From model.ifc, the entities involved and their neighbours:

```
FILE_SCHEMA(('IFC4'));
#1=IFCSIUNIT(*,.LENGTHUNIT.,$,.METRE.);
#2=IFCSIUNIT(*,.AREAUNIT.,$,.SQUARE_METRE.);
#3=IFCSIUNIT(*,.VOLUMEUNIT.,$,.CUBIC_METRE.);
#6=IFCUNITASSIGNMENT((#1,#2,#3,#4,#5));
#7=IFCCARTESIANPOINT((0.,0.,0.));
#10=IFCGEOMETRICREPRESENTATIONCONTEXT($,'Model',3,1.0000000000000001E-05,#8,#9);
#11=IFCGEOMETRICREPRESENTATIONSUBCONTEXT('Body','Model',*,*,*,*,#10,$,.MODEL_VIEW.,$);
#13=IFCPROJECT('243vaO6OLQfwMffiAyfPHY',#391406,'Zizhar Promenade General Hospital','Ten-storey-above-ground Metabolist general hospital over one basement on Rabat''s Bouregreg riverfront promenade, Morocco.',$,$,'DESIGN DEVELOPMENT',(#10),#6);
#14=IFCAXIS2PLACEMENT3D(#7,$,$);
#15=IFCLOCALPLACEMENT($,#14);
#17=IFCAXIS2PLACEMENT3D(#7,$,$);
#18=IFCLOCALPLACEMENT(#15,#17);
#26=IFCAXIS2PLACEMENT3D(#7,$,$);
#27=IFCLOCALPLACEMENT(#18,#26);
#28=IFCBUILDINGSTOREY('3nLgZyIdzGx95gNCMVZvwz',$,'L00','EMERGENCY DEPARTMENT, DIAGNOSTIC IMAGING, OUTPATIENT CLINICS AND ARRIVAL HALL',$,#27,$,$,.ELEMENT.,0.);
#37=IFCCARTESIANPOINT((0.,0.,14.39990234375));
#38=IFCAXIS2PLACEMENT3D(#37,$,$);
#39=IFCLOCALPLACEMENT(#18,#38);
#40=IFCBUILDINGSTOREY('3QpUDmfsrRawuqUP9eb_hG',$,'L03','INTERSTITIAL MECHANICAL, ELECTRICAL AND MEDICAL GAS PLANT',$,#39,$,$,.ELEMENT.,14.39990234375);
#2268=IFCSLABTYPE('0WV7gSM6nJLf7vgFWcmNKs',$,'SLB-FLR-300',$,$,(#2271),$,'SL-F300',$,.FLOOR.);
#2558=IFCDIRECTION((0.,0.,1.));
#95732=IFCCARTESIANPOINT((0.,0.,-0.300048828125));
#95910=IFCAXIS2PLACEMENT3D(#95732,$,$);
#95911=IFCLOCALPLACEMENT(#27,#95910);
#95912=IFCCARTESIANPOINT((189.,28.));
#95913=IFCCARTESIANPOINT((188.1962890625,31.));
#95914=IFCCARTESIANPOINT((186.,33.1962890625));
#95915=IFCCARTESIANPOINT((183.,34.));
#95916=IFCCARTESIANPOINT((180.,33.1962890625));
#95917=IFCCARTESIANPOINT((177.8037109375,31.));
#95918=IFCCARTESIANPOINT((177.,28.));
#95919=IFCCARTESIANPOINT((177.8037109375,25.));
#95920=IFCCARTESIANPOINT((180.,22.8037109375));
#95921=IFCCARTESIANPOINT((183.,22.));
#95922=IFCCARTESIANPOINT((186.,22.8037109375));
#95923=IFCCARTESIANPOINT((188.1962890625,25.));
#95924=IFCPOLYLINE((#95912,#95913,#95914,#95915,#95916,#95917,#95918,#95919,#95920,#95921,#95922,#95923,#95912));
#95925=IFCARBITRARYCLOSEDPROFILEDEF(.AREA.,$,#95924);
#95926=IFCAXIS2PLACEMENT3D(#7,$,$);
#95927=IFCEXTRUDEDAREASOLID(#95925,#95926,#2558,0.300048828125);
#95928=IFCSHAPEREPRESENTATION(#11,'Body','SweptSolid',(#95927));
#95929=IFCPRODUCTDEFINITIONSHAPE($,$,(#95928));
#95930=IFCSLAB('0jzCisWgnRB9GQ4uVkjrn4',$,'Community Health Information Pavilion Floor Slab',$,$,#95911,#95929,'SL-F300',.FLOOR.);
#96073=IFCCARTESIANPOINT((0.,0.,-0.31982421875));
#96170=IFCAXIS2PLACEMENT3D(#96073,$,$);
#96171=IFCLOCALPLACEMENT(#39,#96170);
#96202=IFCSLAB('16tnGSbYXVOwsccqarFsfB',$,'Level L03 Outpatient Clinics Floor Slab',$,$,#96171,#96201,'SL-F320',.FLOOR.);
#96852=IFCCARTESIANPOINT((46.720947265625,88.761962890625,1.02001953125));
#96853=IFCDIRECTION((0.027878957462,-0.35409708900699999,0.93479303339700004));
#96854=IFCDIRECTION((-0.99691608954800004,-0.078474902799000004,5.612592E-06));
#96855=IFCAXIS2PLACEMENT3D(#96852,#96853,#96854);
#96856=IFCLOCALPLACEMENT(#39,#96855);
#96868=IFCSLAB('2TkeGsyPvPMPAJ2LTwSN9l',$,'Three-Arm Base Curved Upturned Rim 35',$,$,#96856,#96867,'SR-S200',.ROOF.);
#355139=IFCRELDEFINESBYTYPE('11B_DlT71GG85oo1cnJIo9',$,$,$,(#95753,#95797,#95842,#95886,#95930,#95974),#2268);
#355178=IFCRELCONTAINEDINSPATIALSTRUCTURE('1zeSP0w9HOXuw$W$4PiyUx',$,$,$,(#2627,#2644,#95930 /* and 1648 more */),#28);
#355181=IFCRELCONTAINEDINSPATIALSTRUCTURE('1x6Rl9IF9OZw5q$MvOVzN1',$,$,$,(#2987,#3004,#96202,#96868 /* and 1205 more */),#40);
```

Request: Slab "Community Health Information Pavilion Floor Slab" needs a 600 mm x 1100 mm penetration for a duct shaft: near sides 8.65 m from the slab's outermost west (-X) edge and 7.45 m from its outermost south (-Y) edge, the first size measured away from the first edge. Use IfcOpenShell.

```python
import numpy as np
import ifcopenshell
import ifcopenshell.api.feature
import ifcopenshell.api.geometry
import ifcopenshell.api.root
import ifcopenshell.geom
import ifcopenshell.util.placement
import ifcopenshell.util.representation
import ifcopenshell.util.shape
import ifcopenshell.util.unit

model = ifcopenshell.open("model.ifc")
unit_scale = ifcopenshell.util.unit.calculate_unit_scale(model)
settings = ifcopenshell.geom.settings()


def volume(element):
    """Net volume in cubic metres, openings subtracted."""
    shape = ifcopenshell.geom.create_shape(settings, element)
    return ifcopenshell.util.shape.get_volume(shape.geometry)


slab = model.by_guid("0jzCisWgnRB9GQ4uVkjrn4")
before = volume(slab)

# Extent in the slab's own axes, in metres. The edges named are its -X and -Y sides.
slab_shape = ifcopenshell.geom.create_shape(settings, slab)
vertices = ifcopenshell.util.shape.get_vertices(slab_shape.geometry)
x_min, y_min, bottom = vertices.min(axis=0)
top = vertices[:, 2].max()

opening = ifcopenshell.api.root.create_entity(model, ifc_class="IfcOpeningElement", name="Duct shaft opening", predefined_type="OPENING")
context = ifcopenshell.util.representation.get_context(model, "Model", "Body", "MODEL_VIEW")
width, depth = 0.6, 1.1
outline = [(0.0, 0.0), (width, 0.0), (width, depth), (0.0, depth), (0.0, 0.0)]
# Overshoot both faces by 50 mm so the cut is clean.
shape = ifcopenshell.api.geometry.add_slab_representation(
    model, context=context, depth=top - bottom + 0.1, polyline=outline
)
ifcopenshell.api.geometry.assign_representation(model, product=opening, representation=shape)

matrix = ifcopenshell.util.placement.get_local_placement(slab.ObjectPlacement)
matrix[:, 3] = matrix @ np.append(np.array([x_min + 8.65, y_min + 7.45, bottom - 0.05]) / unit_scale, 1.0)
ifcopenshell.api.geometry.edit_object_placement(model, product=opening, matrix=matrix, is_si=False)
ifcopenshell.api.feature.add_feature(model, feature=opening, element=slab)

after = volume(slab)

print(f"slab volume {before:.3f} -> {after:.3f} m3")

model.write("model_edited.ifc")
```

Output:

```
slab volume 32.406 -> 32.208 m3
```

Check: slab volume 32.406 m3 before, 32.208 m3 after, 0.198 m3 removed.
